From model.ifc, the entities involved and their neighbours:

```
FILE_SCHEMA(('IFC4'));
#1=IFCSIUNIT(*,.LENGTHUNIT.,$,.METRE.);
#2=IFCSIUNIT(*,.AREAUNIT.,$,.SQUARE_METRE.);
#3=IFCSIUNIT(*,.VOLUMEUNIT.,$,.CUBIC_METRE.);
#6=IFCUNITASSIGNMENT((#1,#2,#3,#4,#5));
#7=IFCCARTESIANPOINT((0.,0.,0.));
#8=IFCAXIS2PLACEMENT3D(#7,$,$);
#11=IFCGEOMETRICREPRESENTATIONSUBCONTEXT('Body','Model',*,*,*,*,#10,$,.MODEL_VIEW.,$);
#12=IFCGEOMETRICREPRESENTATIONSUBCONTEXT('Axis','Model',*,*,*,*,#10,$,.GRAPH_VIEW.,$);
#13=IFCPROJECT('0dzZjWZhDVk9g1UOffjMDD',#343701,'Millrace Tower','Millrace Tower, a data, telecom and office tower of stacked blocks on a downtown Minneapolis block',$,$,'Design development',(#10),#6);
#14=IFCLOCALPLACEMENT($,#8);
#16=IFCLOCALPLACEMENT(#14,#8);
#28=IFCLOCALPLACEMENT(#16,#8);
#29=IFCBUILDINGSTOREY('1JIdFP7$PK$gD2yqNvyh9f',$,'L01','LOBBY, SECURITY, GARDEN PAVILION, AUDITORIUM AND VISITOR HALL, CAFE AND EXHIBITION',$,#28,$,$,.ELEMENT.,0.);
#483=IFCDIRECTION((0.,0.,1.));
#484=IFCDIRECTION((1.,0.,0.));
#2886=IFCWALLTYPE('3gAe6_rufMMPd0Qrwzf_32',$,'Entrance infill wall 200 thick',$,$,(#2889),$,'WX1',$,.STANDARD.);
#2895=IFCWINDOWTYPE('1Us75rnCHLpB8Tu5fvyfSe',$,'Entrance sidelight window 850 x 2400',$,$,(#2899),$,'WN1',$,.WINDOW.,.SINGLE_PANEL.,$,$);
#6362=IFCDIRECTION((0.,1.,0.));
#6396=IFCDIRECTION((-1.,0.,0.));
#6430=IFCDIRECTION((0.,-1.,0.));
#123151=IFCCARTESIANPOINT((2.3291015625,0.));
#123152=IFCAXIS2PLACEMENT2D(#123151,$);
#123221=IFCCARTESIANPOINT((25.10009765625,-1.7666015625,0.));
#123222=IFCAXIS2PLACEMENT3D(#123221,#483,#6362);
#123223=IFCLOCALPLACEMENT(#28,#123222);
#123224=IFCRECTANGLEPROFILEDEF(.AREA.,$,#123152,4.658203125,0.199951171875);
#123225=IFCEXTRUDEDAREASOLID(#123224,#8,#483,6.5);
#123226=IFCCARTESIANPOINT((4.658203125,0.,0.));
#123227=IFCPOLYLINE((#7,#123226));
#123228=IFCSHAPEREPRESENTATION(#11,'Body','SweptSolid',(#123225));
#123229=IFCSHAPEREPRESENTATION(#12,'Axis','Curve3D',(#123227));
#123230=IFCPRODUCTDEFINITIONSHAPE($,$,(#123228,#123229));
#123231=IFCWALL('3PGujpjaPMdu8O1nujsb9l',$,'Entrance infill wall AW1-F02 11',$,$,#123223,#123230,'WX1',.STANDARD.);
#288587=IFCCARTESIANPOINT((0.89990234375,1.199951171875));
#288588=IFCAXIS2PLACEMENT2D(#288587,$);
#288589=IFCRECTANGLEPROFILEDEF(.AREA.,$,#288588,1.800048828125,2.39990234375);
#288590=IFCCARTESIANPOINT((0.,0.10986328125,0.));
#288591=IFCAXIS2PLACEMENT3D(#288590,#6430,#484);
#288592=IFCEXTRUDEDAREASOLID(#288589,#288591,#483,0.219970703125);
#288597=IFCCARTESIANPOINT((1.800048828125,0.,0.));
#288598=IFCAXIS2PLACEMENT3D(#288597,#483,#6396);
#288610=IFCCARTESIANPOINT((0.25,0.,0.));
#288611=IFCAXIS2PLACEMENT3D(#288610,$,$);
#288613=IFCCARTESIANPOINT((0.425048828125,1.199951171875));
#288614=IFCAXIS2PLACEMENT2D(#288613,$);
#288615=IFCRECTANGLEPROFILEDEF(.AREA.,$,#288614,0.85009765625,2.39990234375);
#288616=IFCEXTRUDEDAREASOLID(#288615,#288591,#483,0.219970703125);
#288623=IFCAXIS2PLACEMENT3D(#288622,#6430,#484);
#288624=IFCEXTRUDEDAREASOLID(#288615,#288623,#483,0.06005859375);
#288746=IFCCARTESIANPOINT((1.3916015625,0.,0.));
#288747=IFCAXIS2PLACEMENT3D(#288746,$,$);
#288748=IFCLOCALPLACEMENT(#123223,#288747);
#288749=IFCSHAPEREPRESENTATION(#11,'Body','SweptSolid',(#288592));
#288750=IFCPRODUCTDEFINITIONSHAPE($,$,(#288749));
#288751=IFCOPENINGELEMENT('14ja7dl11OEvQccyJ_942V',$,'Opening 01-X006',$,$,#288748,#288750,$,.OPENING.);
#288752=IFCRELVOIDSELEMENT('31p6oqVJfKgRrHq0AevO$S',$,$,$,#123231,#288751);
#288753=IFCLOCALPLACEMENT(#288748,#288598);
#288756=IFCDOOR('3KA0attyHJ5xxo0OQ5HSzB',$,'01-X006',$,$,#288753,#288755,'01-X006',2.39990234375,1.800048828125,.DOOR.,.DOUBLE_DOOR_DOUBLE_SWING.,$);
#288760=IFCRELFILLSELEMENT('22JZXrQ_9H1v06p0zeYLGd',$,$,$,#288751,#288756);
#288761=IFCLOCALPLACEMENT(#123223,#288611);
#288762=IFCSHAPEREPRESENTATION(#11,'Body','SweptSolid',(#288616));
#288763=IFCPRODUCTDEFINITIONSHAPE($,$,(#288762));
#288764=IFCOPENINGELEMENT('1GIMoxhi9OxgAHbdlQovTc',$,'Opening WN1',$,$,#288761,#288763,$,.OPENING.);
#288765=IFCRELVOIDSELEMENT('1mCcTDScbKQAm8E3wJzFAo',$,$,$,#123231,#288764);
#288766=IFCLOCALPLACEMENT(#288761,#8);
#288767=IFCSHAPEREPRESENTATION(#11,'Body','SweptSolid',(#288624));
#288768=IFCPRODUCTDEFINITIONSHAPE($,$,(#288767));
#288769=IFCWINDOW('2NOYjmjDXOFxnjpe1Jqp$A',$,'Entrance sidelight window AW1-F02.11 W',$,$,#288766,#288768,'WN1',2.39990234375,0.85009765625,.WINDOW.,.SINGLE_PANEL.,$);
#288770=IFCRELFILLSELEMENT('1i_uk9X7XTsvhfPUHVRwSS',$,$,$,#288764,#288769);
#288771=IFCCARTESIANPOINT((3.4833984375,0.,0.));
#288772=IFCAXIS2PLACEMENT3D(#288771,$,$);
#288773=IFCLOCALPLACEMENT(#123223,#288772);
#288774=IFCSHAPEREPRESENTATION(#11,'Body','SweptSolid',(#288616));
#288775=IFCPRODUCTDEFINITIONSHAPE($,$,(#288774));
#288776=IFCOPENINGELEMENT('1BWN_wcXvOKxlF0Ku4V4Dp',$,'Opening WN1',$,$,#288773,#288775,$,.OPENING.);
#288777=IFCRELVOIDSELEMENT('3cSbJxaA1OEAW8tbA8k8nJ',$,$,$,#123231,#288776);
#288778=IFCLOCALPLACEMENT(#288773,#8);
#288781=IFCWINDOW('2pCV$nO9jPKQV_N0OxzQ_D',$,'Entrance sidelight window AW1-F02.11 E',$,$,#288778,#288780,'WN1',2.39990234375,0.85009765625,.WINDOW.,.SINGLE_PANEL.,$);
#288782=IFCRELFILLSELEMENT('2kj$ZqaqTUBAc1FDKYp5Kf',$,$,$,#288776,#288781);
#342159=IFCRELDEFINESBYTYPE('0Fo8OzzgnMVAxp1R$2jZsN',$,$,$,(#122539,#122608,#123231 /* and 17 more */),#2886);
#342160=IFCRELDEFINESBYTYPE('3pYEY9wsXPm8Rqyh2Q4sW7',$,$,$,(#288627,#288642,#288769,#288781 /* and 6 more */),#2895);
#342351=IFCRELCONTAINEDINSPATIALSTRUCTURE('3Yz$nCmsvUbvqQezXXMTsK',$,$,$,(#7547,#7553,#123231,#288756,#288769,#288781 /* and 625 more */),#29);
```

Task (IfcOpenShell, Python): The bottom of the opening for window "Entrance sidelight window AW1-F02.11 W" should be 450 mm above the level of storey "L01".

```python
import numpy as np
import ifcopenshell
import ifcopenshell.api.geometry
import ifcopenshell.geom
import ifcopenshell.util.element
import ifcopenshell.util.placement
import ifcopenshell.util.shape
import ifcopenshell.util.unit

model = ifcopenshell.open("model.ifc")
unit_scale = ifcopenshell.util.unit.calculate_unit_scale(model)

window = model.by_guid("2NOYjmjDXOFxnjpe1Jqp$A")
opening = window.FillsVoids[0].RelatingOpeningElement
storey = ifcopenshell.util.element.get_container(window, ifc_class="IfcBuildingStorey")
level = ifcopenshell.util.placement.get_local_placement(storey.ObjectPlacement)[2, 3]

# The opening's origin need not be at the sill, so measure its lowest point.
shape = ifcopenshell.geom.create_shape(ifcopenshell.geom.settings(), opening)
bottom = ifcopenshell.util.shape.get_shape_bottom_elevation(shape, shape.geometry) / unit_scale
dz = level + 0.45 / unit_scale - bottom

shift = np.array([0.0, 0.0, dz])
# The window is placed relative to its opening, so it follows when the opening moves.
matrix = ifcopenshell.util.placement.get_local_placement(opening.ObjectPlacement)
matrix[:3, 3] += shift
ifcopenshell.api.geometry.edit_object_placement(
    model, product=opening, matrix=matrix, is_si=False, should_transform_children=True
)

print(f"moved by {dz * unit_scale:+.3f} m")

model.write("model_updated.ifc")
```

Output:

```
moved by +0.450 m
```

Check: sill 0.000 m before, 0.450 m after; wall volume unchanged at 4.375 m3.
